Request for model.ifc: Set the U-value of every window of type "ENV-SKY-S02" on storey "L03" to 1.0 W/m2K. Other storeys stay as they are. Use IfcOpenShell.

First a look at what the model holds.

```python
import ifcopenshell
import ifcopenshell.util.element

model = ifcopenshell.open("model.ifc")
print(model.schema)
storey = next(s for s in model.by_type("IfcBuildingStorey") if s.Name == "L03")
windows = [e for e in ifcopenshell.util.element.get_decomposition(storey) if e.is_a("IfcWindow")]
seen = {}
for e in windows:
    element_type = ifcopenshell.util.element.get_type(e)
    key = (element_type.Name if element_type != e and element_type else None, ifcopenshell.util.element.get_pset(e, "Pset_WindowCommon", "ThermalTransmittance"))
    seen[key] = seen.get(key, 0) + 1
for (name, value), count in sorted(seen.items(), key=str):
    print(count, "x", name, "|", value)
```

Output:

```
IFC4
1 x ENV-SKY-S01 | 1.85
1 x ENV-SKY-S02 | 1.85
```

```python
import ifcopenshell
import ifcopenshell.api.pset
import ifcopenshell.util.element

model = ifcopenshell.open("model.ifc")

storey = next(s for s in model.by_type("IfcBuildingStorey") if s.Name == "L03")
windows = [e for e in ifcopenshell.util.element.get_decomposition(storey) if e.is_a("IfcWindow")]

count = 0
for e in windows:
    element_type = ifcopenshell.util.element.get_type(e)
    if element_type in (None, e) or element_type.Name != "ENV-SKY-S02":
        continue
    # add_pset returns the element's existing set when there is one.
    pset = ifcopenshell.api.pset.add_pset(model, product=e, name="Pset_WindowCommon")
    ifcopenshell.api.pset.edit_pset(model, pset=pset, properties={"ThermalTransmittance": 1.0})
    count += 1

print(count, "windows updated")

model.write("model_edited.ifc")
```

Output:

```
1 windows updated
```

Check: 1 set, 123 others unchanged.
